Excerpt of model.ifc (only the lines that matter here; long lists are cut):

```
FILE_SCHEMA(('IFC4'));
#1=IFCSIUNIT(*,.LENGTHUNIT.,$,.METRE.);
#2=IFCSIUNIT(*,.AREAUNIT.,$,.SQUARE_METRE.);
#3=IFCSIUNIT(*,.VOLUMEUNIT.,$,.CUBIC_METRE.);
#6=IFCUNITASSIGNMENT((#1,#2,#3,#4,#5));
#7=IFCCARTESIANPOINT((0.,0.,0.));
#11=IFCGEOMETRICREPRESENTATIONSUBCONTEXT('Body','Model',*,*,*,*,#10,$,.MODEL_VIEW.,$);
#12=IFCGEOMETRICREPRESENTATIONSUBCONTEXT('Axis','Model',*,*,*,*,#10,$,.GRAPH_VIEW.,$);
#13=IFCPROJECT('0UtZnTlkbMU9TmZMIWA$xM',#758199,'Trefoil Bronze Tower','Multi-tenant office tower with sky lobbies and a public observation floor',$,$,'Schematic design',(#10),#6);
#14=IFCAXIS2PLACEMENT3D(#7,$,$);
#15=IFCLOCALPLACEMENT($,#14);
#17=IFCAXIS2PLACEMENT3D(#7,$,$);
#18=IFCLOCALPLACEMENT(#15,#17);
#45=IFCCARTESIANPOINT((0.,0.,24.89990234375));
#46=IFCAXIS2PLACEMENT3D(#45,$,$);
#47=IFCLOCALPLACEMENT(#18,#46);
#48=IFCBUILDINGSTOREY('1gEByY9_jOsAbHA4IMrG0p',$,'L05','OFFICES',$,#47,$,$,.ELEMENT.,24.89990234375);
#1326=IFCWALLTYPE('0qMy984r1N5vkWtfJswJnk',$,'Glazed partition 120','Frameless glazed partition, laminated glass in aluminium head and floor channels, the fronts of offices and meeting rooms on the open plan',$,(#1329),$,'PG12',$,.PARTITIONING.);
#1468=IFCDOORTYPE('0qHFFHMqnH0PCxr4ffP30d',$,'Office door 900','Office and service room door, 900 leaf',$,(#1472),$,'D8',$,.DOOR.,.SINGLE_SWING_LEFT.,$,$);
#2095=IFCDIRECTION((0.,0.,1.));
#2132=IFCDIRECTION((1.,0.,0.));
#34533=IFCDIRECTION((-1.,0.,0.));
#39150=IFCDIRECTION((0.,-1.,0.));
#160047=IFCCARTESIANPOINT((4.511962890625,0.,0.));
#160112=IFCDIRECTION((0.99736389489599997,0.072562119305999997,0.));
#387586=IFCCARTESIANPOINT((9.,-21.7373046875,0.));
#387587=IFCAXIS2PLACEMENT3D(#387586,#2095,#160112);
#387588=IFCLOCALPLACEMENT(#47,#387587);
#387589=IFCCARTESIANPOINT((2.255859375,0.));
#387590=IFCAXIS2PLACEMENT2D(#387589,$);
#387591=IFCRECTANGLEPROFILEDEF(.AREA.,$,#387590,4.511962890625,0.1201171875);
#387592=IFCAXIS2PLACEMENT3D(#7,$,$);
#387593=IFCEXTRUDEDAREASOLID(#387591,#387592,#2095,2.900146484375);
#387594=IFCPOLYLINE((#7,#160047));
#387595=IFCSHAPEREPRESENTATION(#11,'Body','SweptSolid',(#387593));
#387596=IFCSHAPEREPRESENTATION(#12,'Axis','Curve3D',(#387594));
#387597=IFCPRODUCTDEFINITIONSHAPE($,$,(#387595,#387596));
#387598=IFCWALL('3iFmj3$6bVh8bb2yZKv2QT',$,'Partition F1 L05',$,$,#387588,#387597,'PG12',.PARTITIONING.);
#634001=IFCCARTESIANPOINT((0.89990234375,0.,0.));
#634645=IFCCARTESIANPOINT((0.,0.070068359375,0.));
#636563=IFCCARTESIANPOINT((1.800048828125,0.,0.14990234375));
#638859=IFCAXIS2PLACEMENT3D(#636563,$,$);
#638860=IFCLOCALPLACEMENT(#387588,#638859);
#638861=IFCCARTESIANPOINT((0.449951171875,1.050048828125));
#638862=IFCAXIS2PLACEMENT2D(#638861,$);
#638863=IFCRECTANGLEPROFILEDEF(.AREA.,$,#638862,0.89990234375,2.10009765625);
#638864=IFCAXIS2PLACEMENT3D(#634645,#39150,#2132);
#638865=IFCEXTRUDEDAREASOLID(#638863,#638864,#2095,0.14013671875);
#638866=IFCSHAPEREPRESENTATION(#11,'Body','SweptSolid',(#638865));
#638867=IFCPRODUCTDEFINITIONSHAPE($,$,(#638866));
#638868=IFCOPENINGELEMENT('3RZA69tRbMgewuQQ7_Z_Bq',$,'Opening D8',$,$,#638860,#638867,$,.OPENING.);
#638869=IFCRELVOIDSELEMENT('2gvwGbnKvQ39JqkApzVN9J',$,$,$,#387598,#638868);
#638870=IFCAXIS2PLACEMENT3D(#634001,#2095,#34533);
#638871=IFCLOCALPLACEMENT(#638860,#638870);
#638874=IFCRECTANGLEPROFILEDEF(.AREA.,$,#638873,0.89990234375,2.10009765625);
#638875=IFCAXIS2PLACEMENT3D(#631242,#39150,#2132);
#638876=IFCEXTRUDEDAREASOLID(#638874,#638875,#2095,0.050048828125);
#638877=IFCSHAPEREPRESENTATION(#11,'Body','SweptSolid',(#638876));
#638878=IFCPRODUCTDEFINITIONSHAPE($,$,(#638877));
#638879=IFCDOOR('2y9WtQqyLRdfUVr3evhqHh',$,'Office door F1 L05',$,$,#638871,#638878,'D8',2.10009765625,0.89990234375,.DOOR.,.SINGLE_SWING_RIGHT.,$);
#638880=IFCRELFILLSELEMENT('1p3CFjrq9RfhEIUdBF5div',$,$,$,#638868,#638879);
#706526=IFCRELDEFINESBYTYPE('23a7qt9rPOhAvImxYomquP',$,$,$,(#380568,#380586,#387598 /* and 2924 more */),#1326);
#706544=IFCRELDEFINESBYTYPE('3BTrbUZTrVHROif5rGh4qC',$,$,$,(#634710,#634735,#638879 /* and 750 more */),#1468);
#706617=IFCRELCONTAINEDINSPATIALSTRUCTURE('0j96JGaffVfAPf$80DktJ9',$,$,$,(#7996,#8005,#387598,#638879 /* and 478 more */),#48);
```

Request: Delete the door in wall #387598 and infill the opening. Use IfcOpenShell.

```python
import ifcopenshell
import ifcopenshell.api.feature
import ifcopenshell.api.root
import ifcopenshell.geom
import ifcopenshell.util.shape

model = ifcopenshell.open("model.ifc")
settings = ifcopenshell.geom.settings()


def volume(element):
    """Net volume in cubic metres, openings subtracted."""
    shape = ifcopenshell.geom.create_shape(settings, element)
    return ifcopenshell.util.shape.get_volume(shape.geometry)


door = model.by_guid("2y9WtQqyLRdfUVr3evhqHh")
opening = door.FillsVoids[0].RelatingOpeningElement
wall = opening.VoidsElements[0].RelatingBuildingElement
before = volume(wall)

ifcopenshell.api.root.remove_product(model, product=door)
ifcopenshell.api.feature.remove_feature(model, feature=opening)

after = volume(wall)

print(f"wall volume {before:.3f} -> {after:.3f} m3")

model.write("model_updated.ifc")
```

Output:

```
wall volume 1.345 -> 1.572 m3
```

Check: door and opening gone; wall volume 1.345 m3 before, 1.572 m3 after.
